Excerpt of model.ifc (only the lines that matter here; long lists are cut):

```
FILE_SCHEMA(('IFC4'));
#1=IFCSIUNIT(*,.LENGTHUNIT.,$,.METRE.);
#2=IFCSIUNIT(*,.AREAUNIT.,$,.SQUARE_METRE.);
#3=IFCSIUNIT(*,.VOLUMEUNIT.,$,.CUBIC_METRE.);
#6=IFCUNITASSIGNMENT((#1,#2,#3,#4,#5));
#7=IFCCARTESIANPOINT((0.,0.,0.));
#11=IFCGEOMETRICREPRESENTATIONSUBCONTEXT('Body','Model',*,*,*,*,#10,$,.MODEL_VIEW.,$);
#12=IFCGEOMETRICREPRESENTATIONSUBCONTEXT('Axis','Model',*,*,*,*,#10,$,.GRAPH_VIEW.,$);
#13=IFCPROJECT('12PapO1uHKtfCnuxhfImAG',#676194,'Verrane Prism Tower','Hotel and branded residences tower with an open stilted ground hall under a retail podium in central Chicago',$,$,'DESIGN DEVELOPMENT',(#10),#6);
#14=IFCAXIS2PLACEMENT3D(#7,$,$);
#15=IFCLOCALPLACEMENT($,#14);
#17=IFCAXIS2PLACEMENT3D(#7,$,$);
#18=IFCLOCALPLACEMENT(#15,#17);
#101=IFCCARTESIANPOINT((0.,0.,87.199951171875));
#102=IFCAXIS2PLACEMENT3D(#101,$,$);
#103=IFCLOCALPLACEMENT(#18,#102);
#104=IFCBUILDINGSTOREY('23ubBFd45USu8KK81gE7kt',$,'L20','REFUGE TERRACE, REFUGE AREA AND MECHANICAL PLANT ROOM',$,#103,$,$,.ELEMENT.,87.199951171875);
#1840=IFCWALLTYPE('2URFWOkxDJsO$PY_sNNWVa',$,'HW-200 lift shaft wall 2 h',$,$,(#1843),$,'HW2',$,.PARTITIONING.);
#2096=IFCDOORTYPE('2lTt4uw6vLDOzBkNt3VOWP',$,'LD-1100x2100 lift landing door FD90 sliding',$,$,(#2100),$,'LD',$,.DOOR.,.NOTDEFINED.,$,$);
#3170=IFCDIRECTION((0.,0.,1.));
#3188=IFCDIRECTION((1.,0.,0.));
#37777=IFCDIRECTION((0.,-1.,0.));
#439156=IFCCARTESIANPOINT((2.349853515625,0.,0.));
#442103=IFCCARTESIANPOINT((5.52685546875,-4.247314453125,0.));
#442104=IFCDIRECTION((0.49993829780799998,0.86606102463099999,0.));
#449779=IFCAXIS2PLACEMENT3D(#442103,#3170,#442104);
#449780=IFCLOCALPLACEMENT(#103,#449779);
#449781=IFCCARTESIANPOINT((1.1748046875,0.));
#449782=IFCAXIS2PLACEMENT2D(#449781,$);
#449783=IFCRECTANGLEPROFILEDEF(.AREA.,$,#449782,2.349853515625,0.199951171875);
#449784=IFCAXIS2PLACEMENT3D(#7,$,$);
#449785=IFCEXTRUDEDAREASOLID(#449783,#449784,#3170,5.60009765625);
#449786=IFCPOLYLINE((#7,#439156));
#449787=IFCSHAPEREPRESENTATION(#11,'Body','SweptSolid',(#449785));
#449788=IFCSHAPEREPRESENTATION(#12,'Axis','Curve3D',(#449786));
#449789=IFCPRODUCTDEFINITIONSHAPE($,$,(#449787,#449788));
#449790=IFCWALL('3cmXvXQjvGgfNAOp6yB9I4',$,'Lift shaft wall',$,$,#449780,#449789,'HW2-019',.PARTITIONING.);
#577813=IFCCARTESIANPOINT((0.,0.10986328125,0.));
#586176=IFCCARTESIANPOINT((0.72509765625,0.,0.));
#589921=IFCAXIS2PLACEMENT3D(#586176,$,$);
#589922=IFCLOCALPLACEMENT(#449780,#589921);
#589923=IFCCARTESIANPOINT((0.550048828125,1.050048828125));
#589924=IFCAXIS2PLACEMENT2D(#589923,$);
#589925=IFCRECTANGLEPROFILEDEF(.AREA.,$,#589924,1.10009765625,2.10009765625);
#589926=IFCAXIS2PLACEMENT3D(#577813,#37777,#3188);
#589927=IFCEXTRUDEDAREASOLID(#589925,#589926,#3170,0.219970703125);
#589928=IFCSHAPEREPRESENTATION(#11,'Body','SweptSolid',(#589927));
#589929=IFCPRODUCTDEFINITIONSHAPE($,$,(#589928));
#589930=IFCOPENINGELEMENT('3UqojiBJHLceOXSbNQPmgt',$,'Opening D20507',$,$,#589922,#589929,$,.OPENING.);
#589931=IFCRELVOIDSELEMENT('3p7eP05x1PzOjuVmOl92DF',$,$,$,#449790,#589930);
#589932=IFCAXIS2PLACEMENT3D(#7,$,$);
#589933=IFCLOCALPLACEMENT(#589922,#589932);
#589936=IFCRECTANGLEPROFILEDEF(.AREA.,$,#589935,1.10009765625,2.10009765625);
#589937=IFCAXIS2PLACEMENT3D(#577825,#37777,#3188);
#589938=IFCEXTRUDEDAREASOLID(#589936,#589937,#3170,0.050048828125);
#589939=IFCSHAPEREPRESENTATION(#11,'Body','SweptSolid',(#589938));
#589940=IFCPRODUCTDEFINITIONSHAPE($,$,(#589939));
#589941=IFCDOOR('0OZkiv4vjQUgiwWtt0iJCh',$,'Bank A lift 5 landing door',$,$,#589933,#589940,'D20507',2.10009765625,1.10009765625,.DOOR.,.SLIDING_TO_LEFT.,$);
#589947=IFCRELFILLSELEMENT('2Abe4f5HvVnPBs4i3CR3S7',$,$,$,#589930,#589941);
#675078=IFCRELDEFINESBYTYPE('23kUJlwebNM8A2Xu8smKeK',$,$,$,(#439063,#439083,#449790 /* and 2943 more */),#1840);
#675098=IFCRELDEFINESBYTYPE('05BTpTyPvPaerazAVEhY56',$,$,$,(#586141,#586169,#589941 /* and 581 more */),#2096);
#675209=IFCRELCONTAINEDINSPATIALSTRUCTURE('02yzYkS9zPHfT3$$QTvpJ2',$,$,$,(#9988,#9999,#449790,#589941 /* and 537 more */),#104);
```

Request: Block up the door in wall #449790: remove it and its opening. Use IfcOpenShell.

```python
import ifcopenshell
import ifcopenshell.api.feature
import ifcopenshell.api.root
import ifcopenshell.geom
import ifcopenshell.util.shape

model = ifcopenshell.open("model.ifc")
settings = ifcopenshell.geom.settings()


def volume(element):
    """Net volume in cubic metres, openings subtracted."""
    shape = ifcopenshell.geom.create_shape(settings, element)
    return ifcopenshell.util.shape.get_volume(shape.geometry)


door = model.by_guid("0OZkiv4vjQUgiwWtt0iJCh")
opening = door.FillsVoids[0].RelatingOpeningElement
wall = opening.VoidsElements[0].RelatingBuildingElement
before = volume(wall)

ifcopenshell.api.root.remove_product(model, product=door)
ifcopenshell.api.feature.remove_feature(model, feature=opening)

after = volume(wall)

print(f"wall volume {before:.3f} -> {after:.3f} m3")

model.write("model_edited.ifc")
```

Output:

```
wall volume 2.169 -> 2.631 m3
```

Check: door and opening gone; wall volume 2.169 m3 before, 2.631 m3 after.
